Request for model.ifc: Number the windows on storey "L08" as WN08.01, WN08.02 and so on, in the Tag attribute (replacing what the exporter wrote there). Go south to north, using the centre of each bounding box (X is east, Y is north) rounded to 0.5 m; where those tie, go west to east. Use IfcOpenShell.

First a look at what the model holds.

```python
import ifcopenshell
import ifcopenshell.util.element
import ifcopenshell.util.placement

model = ifcopenshell.open("model.ifc")
print(model.schema)
storey = next(s for s in model.by_type("IfcBuildingStorey") if s.Name == "L08")
windows = [e for e in ifcopenshell.util.element.get_decomposition(storey) if e.is_a("IfcWindow")]
for e in sorted(windows, key=lambda e: e.id()):
    origin = ifcopenshell.util.placement.get_local_placement(e.ObjectPlacement)[:3, 3]
    print(e.id(), e.Tag, e.Name, origin.round(2) + 0.0, sep=" | ")
```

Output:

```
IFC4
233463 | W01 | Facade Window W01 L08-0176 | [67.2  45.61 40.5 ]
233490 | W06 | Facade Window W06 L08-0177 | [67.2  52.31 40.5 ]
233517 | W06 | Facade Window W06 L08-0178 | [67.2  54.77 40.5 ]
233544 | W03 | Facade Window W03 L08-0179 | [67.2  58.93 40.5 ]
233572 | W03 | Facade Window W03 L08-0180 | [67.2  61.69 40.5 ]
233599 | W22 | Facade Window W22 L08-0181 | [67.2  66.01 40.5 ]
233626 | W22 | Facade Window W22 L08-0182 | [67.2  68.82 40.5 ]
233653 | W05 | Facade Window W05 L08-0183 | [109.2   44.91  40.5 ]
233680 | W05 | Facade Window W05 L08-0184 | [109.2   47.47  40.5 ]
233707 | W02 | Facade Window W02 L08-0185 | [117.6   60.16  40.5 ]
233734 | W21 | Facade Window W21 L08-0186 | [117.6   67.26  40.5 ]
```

```python
import ifcopenshell
import ifcopenshell.geom
import ifcopenshell.util.element
import ifcopenshell.util.shape

model = ifcopenshell.open("model.ifc")
settings = ifcopenshell.geom.settings()
settings.set("use-world-coords", True)


def centre(element):
    shape = ifcopenshell.geom.create_shape(settings, element)
    return ifcopenshell.util.shape.get_bbox_centroid(shape.geometry)


storey = next(s for s in model.by_type("IfcBuildingStorey") if s.Name == "L08")
windows = [e for e in ifcopenshell.util.element.get_decomposition(storey) if e.is_a("IfcWindow")]

# Insertion points can sit at a corner or the storey origin, so sort by the geometry (in metres).
centres = {e: centre(e) for e in windows}
windows.sort(key=lambda e: (round(centres[e][1] / 0.5), centres[e][0]))

for i, e in enumerate(windows, start=1):
    number = f"WN08.{i:02d}"
    e.Tag = number
    print(e.id(), number)

model.write("model_edited.ifc")
```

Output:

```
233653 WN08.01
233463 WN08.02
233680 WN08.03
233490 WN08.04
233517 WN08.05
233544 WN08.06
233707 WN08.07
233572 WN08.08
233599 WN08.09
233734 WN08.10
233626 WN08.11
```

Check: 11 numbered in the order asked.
